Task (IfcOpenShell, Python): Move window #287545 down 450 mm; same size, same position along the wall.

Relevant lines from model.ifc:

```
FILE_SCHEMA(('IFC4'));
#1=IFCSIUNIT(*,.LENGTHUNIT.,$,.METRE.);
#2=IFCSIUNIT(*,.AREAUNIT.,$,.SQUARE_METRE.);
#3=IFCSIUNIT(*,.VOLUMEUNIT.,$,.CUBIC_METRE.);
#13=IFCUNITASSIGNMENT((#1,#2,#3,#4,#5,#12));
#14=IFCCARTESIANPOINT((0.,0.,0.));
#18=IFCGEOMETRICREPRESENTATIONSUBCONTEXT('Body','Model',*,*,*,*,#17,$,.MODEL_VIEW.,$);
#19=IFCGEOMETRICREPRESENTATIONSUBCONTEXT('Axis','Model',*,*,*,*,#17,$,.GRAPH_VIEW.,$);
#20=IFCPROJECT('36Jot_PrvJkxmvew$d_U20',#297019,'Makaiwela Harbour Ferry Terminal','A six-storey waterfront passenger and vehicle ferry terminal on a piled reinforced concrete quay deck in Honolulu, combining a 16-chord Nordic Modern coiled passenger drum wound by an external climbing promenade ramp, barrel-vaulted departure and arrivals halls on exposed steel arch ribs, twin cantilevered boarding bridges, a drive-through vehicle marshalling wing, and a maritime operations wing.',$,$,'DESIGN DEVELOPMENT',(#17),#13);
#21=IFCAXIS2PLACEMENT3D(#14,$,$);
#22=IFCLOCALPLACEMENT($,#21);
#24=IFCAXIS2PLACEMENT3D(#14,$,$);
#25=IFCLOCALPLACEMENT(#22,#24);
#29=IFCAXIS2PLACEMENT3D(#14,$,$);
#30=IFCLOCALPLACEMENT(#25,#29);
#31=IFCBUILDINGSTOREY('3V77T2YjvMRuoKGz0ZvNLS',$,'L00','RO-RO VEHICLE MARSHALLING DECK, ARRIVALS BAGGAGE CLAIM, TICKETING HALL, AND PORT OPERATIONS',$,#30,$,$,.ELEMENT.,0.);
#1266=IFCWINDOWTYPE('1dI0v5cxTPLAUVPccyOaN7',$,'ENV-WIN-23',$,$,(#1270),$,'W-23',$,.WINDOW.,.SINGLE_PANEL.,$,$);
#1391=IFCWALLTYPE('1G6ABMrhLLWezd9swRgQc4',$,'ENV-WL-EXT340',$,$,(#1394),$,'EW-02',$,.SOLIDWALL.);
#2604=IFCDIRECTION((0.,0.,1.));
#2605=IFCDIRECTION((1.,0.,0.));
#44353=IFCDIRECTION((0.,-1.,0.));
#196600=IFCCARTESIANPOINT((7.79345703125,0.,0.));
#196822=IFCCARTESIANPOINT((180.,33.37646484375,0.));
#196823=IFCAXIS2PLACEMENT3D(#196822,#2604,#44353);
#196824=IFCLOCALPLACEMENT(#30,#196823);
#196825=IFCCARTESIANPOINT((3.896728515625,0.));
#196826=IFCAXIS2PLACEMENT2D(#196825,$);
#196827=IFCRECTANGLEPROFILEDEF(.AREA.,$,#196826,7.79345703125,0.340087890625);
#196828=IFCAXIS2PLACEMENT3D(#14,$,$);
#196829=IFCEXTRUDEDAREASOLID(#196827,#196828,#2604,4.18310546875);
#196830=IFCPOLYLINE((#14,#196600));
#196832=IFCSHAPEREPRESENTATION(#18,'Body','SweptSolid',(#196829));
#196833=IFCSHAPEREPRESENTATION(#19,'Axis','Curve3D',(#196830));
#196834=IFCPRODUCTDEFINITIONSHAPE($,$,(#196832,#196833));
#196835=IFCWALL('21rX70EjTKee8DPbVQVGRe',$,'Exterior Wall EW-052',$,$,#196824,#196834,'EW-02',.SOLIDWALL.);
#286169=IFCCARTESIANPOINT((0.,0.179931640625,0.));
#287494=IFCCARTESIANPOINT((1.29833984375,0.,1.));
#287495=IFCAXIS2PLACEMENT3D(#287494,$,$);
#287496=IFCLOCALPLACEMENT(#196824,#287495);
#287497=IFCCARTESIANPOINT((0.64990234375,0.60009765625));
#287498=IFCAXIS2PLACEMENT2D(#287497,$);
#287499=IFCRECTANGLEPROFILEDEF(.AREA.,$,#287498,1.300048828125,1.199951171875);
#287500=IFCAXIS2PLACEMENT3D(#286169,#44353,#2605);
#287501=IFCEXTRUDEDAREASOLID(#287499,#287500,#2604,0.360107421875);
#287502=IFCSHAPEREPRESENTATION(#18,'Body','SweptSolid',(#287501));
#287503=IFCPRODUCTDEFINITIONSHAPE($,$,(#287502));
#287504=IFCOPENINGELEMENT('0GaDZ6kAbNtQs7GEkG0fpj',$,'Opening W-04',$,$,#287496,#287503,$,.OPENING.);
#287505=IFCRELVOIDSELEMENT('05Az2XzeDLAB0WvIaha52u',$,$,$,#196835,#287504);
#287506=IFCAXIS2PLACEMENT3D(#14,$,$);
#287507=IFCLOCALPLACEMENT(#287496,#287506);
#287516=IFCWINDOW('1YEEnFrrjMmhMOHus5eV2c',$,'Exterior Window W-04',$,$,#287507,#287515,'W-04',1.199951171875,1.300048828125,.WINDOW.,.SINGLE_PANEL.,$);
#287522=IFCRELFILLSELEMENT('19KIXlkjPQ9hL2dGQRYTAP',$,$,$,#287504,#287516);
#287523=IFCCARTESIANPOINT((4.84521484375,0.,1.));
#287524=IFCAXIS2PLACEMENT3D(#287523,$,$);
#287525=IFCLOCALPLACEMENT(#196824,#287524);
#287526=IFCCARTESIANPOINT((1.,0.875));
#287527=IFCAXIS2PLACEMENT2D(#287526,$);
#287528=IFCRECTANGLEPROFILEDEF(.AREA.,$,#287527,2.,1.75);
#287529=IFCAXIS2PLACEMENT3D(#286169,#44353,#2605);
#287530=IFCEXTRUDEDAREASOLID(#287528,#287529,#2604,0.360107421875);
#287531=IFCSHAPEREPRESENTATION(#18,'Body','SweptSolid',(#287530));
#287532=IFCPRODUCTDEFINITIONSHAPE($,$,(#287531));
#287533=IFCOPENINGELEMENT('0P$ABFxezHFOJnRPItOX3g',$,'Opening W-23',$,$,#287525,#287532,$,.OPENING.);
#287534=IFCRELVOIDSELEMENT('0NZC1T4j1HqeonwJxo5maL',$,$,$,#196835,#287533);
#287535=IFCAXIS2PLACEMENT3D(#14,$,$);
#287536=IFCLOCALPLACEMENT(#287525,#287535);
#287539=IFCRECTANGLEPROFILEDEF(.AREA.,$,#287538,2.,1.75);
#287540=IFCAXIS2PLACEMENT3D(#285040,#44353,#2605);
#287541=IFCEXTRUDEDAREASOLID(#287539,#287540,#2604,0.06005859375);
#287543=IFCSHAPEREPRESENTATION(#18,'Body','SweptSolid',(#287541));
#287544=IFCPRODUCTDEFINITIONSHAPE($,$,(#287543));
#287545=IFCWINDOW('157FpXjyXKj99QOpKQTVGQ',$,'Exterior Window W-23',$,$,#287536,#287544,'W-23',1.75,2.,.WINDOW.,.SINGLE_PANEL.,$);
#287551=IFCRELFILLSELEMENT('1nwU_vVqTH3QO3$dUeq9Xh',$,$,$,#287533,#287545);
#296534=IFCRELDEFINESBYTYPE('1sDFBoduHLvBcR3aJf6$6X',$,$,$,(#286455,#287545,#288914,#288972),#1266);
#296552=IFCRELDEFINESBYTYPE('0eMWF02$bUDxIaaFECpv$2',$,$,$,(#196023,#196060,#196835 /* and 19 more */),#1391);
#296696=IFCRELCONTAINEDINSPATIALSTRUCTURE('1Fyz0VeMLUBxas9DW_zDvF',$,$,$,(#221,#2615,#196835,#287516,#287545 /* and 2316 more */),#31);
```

```python
import numpy as np
import ifcopenshell
import ifcopenshell.api.geometry
import ifcopenshell.util.placement
import ifcopenshell.util.unit

model = ifcopenshell.open("model.ifc")
unit_scale = ifcopenshell.util.unit.calculate_unit_scale(model)

window = model.by_guid("157FpXjyXKj99QOpKQTVGQ")
opening = window.FillsVoids[0].RelatingOpeningElement
dz = -0.45 / unit_scale

shift = np.array([0.0, 0.0, dz])
# The window is placed relative to its opening, so it follows when the opening moves.
matrix = ifcopenshell.util.placement.get_local_placement(opening.ObjectPlacement)
matrix[:3, 3] += shift
ifcopenshell.api.geometry.edit_object_placement(
    model, product=opening, matrix=matrix, is_si=False, should_transform_children=True
)

print(f"moved by {dz * unit_scale:+.3f} m")

model.write("model-out.ifc")
```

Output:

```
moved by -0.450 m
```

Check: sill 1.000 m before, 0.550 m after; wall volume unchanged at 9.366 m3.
